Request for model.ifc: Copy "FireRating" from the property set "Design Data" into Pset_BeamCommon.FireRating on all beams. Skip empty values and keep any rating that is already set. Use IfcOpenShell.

First a look at what the model holds.

```python
import ifcopenshell
import ifcopenshell.util.element

model = ifcopenshell.open("model.ifc")
print(model.schema)
beams = model.by_type("IfcBeam")
print(len(beams), "beams")
for e in beams[:8]:
    source = ifcopenshell.util.element.get_pset(e, "Design Data", "FireRating")
    target = ifcopenshell.util.element.get_pset(e, "Pset_BeamCommon", "FireRating")
    print(e.id(), repr(source), repr(target), sep=" | ")
```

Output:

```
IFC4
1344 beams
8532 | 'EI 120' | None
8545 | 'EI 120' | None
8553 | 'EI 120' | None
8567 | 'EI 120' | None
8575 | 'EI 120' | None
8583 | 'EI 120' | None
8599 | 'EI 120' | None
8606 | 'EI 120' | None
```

```python
import ifcopenshell
import ifcopenshell.api.pset
import ifcopenshell.util.element

model = ifcopenshell.open("model.ifc")

count = 0
for e in model.by_type("IfcBeam"):
    value = ifcopenshell.util.element.get_pset(e, "Design Data", "FireRating")
    current = ifcopenshell.util.element.get_pset(e, "Pset_BeamCommon", "FireRating")
    if not value or not value.strip() or current:
        continue
    found = ifcopenshell.util.element.get_pset(e, "Pset_BeamCommon", should_inherit=False)
    if found:
        pset = model.by_id(found["id"])
        if len(ifcopenshell.util.element.get_elements_by_pset(pset)) > 1:
            pset = ifcopenshell.api.pset.unshare_pset(model, products=[e], pset=pset)[0]
    else:
        pset = ifcopenshell.api.pset.add_pset(model, product=e, name="Pset_BeamCommon")
    ifcopenshell.api.pset.edit_pset(model, pset=pset, properties={"FireRating": value})
    count += 1

print(count, "beams updated")

model.write("model_updated.ifc")
```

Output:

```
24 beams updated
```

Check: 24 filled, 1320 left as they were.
